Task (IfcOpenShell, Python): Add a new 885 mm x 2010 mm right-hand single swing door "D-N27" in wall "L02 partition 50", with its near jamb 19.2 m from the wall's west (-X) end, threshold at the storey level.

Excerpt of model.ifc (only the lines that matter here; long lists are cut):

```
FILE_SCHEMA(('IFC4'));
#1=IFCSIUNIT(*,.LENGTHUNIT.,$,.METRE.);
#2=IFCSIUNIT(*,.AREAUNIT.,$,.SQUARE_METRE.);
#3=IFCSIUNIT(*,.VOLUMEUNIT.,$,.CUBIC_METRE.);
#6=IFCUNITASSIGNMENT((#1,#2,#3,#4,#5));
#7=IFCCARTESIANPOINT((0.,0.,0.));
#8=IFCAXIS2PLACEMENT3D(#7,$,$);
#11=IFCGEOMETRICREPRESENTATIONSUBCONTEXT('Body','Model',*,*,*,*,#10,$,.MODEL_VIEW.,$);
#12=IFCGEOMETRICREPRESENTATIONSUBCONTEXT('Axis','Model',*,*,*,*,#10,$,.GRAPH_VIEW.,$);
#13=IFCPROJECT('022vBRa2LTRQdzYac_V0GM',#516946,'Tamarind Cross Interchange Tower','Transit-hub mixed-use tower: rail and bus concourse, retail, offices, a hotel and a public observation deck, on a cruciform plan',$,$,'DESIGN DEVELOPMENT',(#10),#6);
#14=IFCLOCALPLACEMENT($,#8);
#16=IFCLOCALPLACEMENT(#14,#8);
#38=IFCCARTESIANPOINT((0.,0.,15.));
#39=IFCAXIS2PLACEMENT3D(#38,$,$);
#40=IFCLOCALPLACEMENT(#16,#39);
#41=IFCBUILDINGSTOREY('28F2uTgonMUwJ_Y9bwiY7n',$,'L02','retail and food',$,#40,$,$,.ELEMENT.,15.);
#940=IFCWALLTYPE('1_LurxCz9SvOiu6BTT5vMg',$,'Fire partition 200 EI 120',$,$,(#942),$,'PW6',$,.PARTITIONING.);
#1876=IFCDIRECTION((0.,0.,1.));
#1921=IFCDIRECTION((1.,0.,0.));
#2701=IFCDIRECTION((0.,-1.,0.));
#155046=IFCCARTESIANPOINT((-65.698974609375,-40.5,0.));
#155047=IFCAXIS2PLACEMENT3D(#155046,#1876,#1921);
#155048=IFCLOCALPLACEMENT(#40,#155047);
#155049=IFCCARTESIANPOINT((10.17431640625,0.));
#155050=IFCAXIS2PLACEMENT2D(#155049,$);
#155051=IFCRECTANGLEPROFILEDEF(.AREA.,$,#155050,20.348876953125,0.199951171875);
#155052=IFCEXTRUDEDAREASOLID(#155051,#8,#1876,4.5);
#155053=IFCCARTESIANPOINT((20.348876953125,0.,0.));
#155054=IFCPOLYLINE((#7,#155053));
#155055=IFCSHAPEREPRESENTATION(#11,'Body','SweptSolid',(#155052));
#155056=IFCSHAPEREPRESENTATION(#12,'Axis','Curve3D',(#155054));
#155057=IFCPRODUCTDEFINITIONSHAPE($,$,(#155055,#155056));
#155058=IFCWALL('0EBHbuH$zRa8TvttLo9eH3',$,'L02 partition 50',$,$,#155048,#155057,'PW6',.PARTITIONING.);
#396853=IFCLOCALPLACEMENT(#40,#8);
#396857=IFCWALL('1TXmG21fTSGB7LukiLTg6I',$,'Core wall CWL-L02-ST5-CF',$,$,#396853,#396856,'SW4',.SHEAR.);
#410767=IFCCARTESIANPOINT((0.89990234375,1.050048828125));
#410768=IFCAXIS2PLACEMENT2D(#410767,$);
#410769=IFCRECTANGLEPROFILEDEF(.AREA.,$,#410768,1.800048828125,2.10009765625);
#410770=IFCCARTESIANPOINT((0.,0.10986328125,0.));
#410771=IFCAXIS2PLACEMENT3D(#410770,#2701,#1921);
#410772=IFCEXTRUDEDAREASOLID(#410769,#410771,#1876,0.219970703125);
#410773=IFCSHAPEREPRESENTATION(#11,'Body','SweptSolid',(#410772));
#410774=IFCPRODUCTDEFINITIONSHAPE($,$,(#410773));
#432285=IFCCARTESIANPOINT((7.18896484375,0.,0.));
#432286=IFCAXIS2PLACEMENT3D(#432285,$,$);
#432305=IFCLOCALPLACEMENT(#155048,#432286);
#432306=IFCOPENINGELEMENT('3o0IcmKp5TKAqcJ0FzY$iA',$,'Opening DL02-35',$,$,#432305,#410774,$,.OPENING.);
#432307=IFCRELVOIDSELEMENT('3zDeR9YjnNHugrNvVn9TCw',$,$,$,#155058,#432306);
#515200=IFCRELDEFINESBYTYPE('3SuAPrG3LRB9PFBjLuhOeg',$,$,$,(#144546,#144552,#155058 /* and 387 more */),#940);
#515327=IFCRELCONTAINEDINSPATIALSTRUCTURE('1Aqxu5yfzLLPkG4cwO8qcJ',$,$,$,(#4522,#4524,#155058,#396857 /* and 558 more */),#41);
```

```python
import numpy as np
import ifcopenshell
import ifcopenshell.api.feature
import ifcopenshell.api.geometry
import ifcopenshell.api.root
import ifcopenshell.api.spatial
import ifcopenshell.geom
import ifcopenshell.util.element
import ifcopenshell.util.placement
import ifcopenshell.util.representation
import ifcopenshell.util.shape
import ifcopenshell.util.unit

model = ifcopenshell.open("model.ifc")
unit_scale = ifcopenshell.util.unit.calculate_unit_scale(model)
settings = ifcopenshell.geom.settings()


def volume(element):
    """Net volume in cubic metres, openings subtracted."""
    shape = ifcopenshell.geom.create_shape(settings, element)
    return ifcopenshell.util.shape.get_volume(shape.geometry)


wall = model.by_id(155058)
storey = ifcopenshell.util.element.get_container(wall, ifc_class="IfcBuildingStorey")
context = ifcopenshell.util.representation.get_context(model, "Model", "Body", "MODEL_VIEW")
before = volume(wall)

width, height, from_end, sill = 0.885, 2.01, 19.2, 0.0  # metres

# The wall runs along its own X axis, and the end named is its -X end.
wall_shape = ifcopenshell.geom.create_shape(settings, wall)
x, y, z = ifcopenshell.util.shape.get_vertices(wall_shape.geometry).T
start = x.min() + from_end
face, thickness = float(y.min()), float(y.max() - y.min())
wall_matrix = ifcopenshell.util.placement.get_local_placement(wall.ObjectPlacement)
level = ifcopenshell.util.placement.get_local_placement(storey.ObjectPlacement)[2, 3]


def in_wall(x, y):
    """Placement at x, y metres in the wall's axes, at sill height."""
    matrix = wall_matrix.copy()
    matrix[:, 3] = wall_matrix @ np.array([x / unit_scale, y / unit_scale, 0.0, 1.0])
    matrix[2, 3] = level + sill / unit_scale
    return matrix


# Opening: a box that overshoots both wall faces by 50 mm.
opening = ifcopenshell.api.root.create_entity(model, ifc_class="IfcOpeningElement", predefined_type="OPENING")
box = ifcopenshell.api.geometry.add_wall_representation(
    model, context=context, length=width, height=height, thickness=thickness + 0.1
)
ifcopenshell.api.geometry.assign_representation(model, product=opening, representation=box)
ifcopenshell.api.geometry.edit_object_placement(model, product=opening, matrix=in_wall(start, face - 0.05), is_si=False)
ifcopenshell.api.feature.add_feature(model, feature=opening, element=wall)

door = ifcopenshell.api.root.create_entity(model, ifc_class="IfcDoor", name="D-N27", predefined_type="DOOR")
door.OverallWidth, door.OverallHeight = width / unit_scale, height / unit_scale
door.OperationType = "SINGLE_SWING_RIGHT"
body = ifcopenshell.api.geometry.add_door_representation(
    model,
    context=context,
    overall_width=door.OverallWidth,
    overall_height=door.OverallHeight,
    operation_type="SINGLE_SWING_RIGHT",
    lining_properties={"LiningDepth": thickness / unit_scale, "ThresholdDepth": thickness / unit_scale},
)
ifcopenshell.api.geometry.assign_representation(model, product=door, representation=body)
ifcopenshell.api.spatial.assign_container(model, products=[door], relating_structure=storey)
ifcopenshell.api.feature.add_filling(model, opening=opening, element=door)

# The lining spans the wall, so the door starts at the wall face.
ifcopenshell.api.geometry.edit_object_placement(model, product=door, matrix=in_wall(start, face), is_si=False)

after = volume(wall)

print(f"wall volume {before:.3f} -> {after:.3f} m3")

model.write("model_rev.ifc")
```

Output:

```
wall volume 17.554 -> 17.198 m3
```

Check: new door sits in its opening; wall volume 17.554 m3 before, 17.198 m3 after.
